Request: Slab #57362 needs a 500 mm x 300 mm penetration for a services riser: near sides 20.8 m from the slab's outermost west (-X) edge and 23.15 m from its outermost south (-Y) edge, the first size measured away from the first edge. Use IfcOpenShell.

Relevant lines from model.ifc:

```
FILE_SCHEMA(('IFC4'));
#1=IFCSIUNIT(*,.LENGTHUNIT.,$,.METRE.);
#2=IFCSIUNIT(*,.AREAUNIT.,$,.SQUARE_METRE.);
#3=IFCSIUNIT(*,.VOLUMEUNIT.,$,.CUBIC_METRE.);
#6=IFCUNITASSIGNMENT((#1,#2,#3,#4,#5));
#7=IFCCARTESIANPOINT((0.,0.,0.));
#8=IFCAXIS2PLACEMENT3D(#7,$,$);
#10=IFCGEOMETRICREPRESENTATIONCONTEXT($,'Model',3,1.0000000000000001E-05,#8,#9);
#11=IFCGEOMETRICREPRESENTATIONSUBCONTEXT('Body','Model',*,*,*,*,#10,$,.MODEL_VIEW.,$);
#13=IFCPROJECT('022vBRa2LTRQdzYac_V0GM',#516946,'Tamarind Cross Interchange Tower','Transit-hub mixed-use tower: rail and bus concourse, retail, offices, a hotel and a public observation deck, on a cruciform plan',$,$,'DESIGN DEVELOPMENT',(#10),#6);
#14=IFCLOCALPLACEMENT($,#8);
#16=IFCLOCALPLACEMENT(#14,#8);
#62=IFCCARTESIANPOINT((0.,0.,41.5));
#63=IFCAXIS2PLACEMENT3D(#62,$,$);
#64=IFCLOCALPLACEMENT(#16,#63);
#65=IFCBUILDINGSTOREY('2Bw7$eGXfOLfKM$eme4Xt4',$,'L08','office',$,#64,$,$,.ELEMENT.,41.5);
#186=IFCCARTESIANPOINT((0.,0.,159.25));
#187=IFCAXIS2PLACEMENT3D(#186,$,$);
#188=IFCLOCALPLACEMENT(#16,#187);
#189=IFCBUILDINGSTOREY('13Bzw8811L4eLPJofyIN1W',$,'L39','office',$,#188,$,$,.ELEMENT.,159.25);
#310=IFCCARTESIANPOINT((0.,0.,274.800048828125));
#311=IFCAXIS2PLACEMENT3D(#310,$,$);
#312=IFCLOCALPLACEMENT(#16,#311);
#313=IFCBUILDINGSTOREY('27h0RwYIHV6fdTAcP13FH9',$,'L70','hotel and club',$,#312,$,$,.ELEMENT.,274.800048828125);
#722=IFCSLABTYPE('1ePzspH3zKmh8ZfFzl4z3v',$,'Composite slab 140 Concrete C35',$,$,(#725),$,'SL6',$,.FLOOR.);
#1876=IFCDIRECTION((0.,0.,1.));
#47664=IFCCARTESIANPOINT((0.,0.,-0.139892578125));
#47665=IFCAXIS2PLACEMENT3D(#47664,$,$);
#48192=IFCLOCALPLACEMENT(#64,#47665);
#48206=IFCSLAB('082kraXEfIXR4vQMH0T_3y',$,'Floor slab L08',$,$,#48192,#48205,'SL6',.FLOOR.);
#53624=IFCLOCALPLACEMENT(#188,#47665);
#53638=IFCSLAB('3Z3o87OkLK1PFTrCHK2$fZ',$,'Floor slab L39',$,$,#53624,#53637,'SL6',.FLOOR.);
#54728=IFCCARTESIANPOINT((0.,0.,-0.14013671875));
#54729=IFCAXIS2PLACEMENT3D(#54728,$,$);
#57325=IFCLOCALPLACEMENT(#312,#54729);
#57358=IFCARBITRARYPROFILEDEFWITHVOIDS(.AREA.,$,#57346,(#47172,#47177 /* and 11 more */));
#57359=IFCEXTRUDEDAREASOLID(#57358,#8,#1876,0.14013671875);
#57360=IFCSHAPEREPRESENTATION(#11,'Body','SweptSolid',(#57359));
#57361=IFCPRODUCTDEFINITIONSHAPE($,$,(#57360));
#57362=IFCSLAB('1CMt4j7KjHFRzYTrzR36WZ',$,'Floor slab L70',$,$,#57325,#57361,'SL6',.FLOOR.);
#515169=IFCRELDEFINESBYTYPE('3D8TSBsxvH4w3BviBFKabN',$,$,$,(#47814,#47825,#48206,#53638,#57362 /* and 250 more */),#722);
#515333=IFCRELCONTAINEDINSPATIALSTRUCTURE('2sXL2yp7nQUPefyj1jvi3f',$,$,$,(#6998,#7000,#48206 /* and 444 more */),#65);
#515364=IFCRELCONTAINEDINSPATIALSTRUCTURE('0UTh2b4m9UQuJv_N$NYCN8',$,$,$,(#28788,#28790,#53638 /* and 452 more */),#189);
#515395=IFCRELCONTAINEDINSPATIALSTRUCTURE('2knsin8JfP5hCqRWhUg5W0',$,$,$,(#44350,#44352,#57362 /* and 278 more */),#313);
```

```python
import numpy as np
import ifcopenshell
import ifcopenshell.api.feature
import ifcopenshell.api.geometry
import ifcopenshell.api.root
import ifcopenshell.geom
import ifcopenshell.util.placement
import ifcopenshell.util.representation
import ifcopenshell.util.shape
import ifcopenshell.util.unit

model = ifcopenshell.open("model.ifc")
unit_scale = ifcopenshell.util.unit.calculate_unit_scale(model)
settings = ifcopenshell.geom.settings()


def volume(element):
    """Net volume in cubic metres, openings subtracted."""
    shape = ifcopenshell.geom.create_shape(settings, element)
    return ifcopenshell.util.shape.get_volume(shape.geometry)


slab = model.by_guid("1CMt4j7KjHFRzYTrzR36WZ")
before = volume(slab)

# Extent in the slab's own axes, in metres. The edges named are its -X and -Y sides.
slab_shape = ifcopenshell.geom.create_shape(settings, slab)
vertices = ifcopenshell.util.shape.get_vertices(slab_shape.geometry)
x_min, y_min, bottom = vertices.min(axis=0)
top = vertices[:, 2].max()

opening = ifcopenshell.api.root.create_entity(model, ifc_class="IfcOpeningElement", name="Services riser opening", predefined_type="OPENING")
context = ifcopenshell.util.representation.get_context(model, "Model", "Body", "MODEL_VIEW")
width, depth = 0.5, 0.3
outline = [(0.0, 0.0), (width, 0.0), (width, depth), (0.0, depth), (0.0, 0.0)]
# Overshoot both faces by 50 mm so the cut is clean.
shape = ifcopenshell.api.geometry.add_slab_representation(
    model, context=context, depth=top - bottom + 0.1, polyline=outline
)
ifcopenshell.api.geometry.assign_representation(model, product=opening, representation=shape)

matrix = ifcopenshell.util.placement.get_local_placement(slab.ObjectPlacement)
matrix[:, 3] = matrix @ np.append(np.array([x_min + 20.8, y_min + 23.15, bottom - 0.05]) / unit_scale, 1.0)
ifcopenshell.api.geometry.edit_object_placement(model, product=opening, matrix=matrix, is_si=False)
ifcopenshell.api.feature.add_feature(model, feature=opening, element=slab)

after = volume(slab)

print(f"slab volume {before:.3f} -> {after:.3f} m3")

model.write("model_updated.ifc")
```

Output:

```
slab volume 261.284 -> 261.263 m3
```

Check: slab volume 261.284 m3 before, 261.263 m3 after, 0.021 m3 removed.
